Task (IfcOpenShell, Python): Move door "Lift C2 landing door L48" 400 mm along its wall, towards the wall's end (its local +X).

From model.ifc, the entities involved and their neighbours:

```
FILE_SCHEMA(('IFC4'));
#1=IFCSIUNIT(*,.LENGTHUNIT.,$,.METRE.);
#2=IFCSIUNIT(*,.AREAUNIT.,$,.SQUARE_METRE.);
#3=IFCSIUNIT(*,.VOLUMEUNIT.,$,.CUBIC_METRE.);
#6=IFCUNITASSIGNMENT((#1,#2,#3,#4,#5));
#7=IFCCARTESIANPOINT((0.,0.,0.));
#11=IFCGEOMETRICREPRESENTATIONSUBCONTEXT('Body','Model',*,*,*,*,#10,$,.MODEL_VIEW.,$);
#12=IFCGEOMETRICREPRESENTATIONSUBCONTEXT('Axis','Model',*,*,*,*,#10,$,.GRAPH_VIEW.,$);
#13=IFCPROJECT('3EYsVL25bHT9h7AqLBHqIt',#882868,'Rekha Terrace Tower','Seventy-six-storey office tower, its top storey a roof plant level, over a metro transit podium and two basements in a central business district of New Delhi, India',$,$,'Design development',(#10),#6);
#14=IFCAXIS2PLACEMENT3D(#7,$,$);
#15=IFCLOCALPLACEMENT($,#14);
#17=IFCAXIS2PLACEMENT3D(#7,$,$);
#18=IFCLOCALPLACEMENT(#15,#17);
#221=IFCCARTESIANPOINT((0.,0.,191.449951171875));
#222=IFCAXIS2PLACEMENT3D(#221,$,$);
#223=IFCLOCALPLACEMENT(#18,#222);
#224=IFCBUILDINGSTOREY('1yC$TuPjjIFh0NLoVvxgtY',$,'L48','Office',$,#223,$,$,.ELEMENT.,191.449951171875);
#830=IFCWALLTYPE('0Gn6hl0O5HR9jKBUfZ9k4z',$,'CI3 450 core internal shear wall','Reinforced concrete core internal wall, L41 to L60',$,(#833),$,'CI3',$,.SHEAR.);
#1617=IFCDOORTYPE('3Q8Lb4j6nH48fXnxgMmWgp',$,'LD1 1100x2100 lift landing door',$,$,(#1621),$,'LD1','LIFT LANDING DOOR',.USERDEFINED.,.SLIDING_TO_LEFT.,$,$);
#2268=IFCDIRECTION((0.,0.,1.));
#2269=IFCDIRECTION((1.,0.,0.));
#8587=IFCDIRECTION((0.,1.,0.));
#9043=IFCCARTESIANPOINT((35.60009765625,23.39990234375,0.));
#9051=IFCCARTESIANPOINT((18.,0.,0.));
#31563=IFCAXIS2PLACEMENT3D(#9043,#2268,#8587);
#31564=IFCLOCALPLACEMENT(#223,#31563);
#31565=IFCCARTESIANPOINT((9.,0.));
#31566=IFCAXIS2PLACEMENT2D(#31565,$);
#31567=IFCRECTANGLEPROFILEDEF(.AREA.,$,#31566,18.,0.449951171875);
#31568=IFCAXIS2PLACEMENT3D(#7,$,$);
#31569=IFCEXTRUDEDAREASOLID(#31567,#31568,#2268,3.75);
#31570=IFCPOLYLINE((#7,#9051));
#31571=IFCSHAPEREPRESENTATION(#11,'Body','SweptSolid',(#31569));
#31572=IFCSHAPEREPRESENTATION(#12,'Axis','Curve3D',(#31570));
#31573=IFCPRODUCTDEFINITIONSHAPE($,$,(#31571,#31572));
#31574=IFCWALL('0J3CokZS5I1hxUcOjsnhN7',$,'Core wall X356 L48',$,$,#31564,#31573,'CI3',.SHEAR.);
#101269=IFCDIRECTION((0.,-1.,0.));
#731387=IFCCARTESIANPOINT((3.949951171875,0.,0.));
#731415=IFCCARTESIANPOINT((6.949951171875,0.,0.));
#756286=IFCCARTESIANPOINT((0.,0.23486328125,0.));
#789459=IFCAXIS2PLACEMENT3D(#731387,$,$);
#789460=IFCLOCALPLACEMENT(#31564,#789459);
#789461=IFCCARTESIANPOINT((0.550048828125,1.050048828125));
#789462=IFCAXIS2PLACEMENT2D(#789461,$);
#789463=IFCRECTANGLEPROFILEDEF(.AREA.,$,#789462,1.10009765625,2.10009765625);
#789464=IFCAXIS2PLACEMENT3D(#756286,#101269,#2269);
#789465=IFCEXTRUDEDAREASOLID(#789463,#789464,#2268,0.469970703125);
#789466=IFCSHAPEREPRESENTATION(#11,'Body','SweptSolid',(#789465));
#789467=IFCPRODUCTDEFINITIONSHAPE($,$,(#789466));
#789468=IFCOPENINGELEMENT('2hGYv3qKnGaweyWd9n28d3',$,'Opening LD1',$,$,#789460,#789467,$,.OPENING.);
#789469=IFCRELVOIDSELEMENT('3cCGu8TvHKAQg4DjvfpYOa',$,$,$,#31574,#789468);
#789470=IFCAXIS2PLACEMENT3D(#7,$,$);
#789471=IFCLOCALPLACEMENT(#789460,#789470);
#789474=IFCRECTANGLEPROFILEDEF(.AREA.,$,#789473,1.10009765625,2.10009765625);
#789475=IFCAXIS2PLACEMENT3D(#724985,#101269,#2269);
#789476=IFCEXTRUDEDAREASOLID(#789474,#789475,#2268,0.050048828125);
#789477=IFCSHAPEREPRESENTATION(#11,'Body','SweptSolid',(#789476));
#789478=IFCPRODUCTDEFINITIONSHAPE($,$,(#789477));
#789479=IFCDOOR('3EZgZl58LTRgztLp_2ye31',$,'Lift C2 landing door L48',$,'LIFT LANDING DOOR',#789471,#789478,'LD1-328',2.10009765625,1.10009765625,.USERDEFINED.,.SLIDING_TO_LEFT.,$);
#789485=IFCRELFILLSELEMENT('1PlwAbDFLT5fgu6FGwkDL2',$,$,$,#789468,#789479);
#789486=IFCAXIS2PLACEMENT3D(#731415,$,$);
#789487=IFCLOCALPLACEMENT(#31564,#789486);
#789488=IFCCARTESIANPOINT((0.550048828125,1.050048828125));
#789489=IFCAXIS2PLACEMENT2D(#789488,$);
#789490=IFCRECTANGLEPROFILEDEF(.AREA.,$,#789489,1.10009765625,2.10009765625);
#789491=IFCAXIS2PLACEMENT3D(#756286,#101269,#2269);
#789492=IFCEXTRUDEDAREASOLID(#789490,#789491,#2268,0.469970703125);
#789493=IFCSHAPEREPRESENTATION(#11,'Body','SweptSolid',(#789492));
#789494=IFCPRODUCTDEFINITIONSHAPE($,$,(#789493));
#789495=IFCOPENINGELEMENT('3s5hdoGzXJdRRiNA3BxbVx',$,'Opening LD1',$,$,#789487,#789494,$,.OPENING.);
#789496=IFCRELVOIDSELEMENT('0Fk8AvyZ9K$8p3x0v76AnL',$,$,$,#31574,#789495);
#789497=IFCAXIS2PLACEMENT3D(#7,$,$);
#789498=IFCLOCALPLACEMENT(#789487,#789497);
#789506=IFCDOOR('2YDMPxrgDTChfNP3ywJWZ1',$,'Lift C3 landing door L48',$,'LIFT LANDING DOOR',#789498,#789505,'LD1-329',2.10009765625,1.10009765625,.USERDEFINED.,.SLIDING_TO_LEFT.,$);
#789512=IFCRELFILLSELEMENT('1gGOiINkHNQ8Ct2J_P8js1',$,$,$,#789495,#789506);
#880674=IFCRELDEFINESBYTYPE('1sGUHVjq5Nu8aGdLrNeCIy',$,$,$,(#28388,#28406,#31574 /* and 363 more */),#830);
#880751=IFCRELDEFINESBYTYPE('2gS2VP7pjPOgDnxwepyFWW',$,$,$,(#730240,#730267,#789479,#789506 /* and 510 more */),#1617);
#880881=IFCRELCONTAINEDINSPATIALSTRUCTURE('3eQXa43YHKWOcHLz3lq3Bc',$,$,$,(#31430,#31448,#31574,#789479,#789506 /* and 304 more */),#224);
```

```python
import ifcopenshell
import ifcopenshell.api.geometry
import ifcopenshell.util.placement
import ifcopenshell.util.unit

model = ifcopenshell.open("model.ifc")
unit_scale = ifcopenshell.util.unit.calculate_unit_scale(model)

door = model.by_guid("3EZgZl58LTRgztLp_2ye31")
opening = door.FillsVoids[0].RelatingOpeningElement
wall = opening.VoidsElements[0].RelatingBuildingElement

wall_matrix = ifcopenshell.util.placement.get_local_placement(wall.ObjectPlacement)
shift = wall_matrix[:3, 0] * 0.4 / unit_scale
before = ifcopenshell.util.placement.get_local_placement(door.ObjectPlacement)[:3, 3].copy()

# The door is placed relative to its opening, so it follows when the opening moves.
matrix = ifcopenshell.util.placement.get_local_placement(opening.ObjectPlacement)
matrix[:3, 3] += shift
ifcopenshell.api.geometry.edit_object_placement(
    model, product=opening, matrix=matrix, is_si=False, should_transform_children=True
)

after = ifcopenshell.util.placement.get_local_placement(door.ObjectPlacement)[:3, 3]
print("door moved by", (after - before).round(3) + 0.0)

model.write("model_edited.ifc")
```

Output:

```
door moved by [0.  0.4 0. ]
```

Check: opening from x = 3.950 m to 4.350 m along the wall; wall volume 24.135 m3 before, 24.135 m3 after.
